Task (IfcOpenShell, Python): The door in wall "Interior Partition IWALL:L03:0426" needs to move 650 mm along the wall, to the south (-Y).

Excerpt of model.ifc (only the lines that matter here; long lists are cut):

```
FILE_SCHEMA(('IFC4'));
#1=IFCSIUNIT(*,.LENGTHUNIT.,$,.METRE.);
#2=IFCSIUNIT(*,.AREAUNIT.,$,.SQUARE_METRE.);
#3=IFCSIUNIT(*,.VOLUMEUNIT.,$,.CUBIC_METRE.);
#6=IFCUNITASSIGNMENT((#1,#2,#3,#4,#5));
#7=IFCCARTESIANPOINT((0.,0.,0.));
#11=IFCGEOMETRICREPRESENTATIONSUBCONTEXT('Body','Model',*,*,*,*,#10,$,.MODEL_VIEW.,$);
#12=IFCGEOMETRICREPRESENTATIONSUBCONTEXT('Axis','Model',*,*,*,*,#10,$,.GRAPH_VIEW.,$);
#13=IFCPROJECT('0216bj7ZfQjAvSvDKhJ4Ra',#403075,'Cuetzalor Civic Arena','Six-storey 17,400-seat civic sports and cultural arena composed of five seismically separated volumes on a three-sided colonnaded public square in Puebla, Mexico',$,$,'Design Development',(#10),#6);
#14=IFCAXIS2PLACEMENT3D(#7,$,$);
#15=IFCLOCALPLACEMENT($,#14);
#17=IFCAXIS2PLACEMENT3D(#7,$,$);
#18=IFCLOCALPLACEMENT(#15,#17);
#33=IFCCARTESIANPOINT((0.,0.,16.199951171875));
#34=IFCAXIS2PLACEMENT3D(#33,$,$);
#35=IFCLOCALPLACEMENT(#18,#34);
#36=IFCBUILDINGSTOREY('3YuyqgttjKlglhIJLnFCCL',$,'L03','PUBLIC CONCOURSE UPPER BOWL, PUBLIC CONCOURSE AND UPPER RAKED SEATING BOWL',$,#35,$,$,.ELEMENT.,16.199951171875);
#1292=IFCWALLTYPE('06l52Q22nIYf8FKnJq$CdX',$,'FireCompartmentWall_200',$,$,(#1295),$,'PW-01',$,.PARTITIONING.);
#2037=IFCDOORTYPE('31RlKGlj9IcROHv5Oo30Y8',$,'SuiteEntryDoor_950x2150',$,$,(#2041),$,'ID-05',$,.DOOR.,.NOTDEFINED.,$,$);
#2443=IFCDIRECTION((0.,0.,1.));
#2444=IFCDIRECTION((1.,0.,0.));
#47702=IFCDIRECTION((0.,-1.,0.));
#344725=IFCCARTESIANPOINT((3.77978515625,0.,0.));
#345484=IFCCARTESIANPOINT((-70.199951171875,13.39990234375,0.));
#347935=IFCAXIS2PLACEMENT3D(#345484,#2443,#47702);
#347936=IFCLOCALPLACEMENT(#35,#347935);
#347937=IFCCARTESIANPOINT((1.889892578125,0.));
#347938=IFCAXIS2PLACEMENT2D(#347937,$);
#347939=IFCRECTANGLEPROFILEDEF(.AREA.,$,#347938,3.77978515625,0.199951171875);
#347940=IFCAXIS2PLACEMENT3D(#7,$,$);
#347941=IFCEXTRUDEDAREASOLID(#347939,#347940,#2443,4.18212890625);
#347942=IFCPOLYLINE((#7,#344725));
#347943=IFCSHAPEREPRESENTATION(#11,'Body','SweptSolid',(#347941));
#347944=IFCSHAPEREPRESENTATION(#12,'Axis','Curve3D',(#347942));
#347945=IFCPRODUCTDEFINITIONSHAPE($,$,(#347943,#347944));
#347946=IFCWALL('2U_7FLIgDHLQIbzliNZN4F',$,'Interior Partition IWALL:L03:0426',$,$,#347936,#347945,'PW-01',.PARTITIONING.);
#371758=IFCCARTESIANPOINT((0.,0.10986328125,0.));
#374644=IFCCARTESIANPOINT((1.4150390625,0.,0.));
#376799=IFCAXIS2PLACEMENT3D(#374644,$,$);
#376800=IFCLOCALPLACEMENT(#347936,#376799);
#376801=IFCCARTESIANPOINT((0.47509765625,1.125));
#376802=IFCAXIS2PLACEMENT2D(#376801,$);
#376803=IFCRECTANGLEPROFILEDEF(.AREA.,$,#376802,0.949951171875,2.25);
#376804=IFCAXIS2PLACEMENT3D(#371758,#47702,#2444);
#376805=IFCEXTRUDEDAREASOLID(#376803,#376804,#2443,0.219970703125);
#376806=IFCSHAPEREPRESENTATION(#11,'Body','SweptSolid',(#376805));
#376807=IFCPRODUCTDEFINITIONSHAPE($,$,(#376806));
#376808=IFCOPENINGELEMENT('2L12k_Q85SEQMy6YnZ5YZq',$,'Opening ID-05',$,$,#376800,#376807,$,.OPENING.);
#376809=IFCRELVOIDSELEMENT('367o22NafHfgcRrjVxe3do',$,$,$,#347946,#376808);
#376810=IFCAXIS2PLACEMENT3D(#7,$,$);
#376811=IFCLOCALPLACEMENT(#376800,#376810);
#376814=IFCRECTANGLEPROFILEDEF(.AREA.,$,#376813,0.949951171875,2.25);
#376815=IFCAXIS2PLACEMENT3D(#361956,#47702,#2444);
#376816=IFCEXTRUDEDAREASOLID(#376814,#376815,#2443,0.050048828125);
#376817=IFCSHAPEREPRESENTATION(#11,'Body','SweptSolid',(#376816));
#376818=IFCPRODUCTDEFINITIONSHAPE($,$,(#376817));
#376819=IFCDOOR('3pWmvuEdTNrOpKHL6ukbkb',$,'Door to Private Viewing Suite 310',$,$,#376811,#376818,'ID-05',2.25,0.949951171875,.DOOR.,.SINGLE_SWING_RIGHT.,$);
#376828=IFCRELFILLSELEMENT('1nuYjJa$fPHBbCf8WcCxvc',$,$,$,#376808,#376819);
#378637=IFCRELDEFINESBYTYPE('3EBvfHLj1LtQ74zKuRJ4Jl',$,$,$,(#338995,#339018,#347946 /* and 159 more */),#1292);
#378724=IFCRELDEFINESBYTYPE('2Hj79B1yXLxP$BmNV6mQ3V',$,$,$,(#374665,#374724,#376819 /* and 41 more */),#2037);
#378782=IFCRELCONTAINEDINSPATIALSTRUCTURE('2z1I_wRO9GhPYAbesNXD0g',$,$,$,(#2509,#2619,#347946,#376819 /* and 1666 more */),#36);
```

```python
import ifcopenshell
import ifcopenshell.api.geometry
import ifcopenshell.util.placement

model = ifcopenshell.open("model.ifc")

door = model.by_guid("3pWmvuEdTNrOpKHL6ukbkb")
opening = door.FillsVoids[0].RelatingOpeningElement
wall = opening.VoidsElements[0].RelatingBuildingElement

wall_matrix = ifcopenshell.util.placement.get_local_placement(wall.ObjectPlacement)
shift = wall_matrix[:3, 0] * 0.65
before = ifcopenshell.util.placement.get_local_placement(door.ObjectPlacement)[:3, 3].copy()

# The door is placed relative to its opening, so it follows when the opening moves.
matrix = ifcopenshell.util.placement.get_local_placement(opening.ObjectPlacement)
matrix[:3, 3] += shift
ifcopenshell.api.geometry.edit_object_placement(
    model, product=opening, matrix=matrix, is_si=False, should_transform_children=True
)

after = ifcopenshell.util.placement.get_local_placement(door.ObjectPlacement)[:3, 3]
print("door moved by", (after - before).round(3) + 0.0)

model.write("model_edited.ifc")
```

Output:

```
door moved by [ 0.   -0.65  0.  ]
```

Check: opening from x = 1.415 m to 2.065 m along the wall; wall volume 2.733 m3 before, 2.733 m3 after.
